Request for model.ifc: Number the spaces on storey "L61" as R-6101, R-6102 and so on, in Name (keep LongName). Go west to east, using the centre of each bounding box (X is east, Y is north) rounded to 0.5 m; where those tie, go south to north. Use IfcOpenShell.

First a look at what the model holds.

```python
import ifcopenshell
import ifcopenshell.util.element
import ifcopenshell.util.placement

model = ifcopenshell.open("model.ifc")
print(model.schema)
storey = next(s for s in model.by_type("IfcBuildingStorey") if s.Name == "L61")
spaces = [e for e in ifcopenshell.util.element.get_decomposition(storey) if e.is_a("IfcSpace")]
for e in sorted(spaces, key=lambda e: e.id()):
    origin = ifcopenshell.util.placement.get_local_placement(e.ObjectPlacement)[:3, 3]
    print(e.id(), e.Name, e.LongName, origin.round(2) + 0.0, sep=" | ")
```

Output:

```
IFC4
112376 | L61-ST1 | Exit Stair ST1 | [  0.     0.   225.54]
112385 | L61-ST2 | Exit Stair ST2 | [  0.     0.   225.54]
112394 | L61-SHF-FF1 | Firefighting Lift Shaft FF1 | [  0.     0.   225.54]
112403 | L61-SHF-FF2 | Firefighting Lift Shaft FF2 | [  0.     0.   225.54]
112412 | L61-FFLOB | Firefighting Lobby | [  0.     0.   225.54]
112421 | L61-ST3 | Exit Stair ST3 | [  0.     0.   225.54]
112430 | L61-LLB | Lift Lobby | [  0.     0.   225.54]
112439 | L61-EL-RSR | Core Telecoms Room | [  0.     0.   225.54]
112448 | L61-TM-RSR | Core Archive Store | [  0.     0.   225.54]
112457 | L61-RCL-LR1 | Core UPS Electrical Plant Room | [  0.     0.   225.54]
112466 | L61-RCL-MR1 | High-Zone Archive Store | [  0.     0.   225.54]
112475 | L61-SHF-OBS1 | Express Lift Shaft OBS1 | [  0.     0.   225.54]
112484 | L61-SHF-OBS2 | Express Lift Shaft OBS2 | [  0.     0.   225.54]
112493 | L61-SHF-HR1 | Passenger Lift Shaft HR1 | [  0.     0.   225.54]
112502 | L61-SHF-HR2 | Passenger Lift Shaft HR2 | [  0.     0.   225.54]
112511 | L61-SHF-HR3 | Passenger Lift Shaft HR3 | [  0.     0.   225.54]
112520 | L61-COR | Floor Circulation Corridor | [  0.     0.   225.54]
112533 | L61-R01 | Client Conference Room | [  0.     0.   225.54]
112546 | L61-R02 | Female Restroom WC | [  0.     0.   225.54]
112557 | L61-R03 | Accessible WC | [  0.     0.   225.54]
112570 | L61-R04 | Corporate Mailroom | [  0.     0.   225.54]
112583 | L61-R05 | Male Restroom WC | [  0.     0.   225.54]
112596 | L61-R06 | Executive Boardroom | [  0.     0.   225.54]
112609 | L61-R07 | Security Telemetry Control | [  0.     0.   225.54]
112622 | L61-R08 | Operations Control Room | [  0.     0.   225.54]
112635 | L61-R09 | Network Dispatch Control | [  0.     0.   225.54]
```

```python
import ifcopenshell
import ifcopenshell.geom
import ifcopenshell.util.element
import ifcopenshell.util.shape

model = ifcopenshell.open("model.ifc")
settings = ifcopenshell.geom.settings()
settings.set("use-world-coords", True)


def centre(element):
    shape = ifcopenshell.geom.create_shape(settings, element)
    return ifcopenshell.util.shape.get_bbox_centroid(shape.geometry)


storey = next(s for s in model.by_type("IfcBuildingStorey") if s.Name == "L61")
spaces = [e for e in ifcopenshell.util.element.get_decomposition(storey) if e.is_a("IfcSpace")]

# Insertion points can sit at a corner or the storey origin, so sort by the geometry (in metres).
centres = {e: centre(e) for e in spaces}
spaces.sort(key=lambda e: (round(centres[e][0] / 0.5), centres[e][1]))

for i, e in enumerate(spaces, start=1):
    number = f"R-61{i:02d}"
    e.Name = number
    print(e.id(), number)

model.write("model_rev.ifc")
```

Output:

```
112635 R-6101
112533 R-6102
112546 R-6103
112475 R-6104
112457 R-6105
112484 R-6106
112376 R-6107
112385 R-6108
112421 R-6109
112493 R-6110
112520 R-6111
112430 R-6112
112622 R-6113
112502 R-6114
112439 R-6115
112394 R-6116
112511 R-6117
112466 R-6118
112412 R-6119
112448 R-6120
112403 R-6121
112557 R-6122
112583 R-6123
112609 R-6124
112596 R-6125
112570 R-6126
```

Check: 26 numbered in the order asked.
